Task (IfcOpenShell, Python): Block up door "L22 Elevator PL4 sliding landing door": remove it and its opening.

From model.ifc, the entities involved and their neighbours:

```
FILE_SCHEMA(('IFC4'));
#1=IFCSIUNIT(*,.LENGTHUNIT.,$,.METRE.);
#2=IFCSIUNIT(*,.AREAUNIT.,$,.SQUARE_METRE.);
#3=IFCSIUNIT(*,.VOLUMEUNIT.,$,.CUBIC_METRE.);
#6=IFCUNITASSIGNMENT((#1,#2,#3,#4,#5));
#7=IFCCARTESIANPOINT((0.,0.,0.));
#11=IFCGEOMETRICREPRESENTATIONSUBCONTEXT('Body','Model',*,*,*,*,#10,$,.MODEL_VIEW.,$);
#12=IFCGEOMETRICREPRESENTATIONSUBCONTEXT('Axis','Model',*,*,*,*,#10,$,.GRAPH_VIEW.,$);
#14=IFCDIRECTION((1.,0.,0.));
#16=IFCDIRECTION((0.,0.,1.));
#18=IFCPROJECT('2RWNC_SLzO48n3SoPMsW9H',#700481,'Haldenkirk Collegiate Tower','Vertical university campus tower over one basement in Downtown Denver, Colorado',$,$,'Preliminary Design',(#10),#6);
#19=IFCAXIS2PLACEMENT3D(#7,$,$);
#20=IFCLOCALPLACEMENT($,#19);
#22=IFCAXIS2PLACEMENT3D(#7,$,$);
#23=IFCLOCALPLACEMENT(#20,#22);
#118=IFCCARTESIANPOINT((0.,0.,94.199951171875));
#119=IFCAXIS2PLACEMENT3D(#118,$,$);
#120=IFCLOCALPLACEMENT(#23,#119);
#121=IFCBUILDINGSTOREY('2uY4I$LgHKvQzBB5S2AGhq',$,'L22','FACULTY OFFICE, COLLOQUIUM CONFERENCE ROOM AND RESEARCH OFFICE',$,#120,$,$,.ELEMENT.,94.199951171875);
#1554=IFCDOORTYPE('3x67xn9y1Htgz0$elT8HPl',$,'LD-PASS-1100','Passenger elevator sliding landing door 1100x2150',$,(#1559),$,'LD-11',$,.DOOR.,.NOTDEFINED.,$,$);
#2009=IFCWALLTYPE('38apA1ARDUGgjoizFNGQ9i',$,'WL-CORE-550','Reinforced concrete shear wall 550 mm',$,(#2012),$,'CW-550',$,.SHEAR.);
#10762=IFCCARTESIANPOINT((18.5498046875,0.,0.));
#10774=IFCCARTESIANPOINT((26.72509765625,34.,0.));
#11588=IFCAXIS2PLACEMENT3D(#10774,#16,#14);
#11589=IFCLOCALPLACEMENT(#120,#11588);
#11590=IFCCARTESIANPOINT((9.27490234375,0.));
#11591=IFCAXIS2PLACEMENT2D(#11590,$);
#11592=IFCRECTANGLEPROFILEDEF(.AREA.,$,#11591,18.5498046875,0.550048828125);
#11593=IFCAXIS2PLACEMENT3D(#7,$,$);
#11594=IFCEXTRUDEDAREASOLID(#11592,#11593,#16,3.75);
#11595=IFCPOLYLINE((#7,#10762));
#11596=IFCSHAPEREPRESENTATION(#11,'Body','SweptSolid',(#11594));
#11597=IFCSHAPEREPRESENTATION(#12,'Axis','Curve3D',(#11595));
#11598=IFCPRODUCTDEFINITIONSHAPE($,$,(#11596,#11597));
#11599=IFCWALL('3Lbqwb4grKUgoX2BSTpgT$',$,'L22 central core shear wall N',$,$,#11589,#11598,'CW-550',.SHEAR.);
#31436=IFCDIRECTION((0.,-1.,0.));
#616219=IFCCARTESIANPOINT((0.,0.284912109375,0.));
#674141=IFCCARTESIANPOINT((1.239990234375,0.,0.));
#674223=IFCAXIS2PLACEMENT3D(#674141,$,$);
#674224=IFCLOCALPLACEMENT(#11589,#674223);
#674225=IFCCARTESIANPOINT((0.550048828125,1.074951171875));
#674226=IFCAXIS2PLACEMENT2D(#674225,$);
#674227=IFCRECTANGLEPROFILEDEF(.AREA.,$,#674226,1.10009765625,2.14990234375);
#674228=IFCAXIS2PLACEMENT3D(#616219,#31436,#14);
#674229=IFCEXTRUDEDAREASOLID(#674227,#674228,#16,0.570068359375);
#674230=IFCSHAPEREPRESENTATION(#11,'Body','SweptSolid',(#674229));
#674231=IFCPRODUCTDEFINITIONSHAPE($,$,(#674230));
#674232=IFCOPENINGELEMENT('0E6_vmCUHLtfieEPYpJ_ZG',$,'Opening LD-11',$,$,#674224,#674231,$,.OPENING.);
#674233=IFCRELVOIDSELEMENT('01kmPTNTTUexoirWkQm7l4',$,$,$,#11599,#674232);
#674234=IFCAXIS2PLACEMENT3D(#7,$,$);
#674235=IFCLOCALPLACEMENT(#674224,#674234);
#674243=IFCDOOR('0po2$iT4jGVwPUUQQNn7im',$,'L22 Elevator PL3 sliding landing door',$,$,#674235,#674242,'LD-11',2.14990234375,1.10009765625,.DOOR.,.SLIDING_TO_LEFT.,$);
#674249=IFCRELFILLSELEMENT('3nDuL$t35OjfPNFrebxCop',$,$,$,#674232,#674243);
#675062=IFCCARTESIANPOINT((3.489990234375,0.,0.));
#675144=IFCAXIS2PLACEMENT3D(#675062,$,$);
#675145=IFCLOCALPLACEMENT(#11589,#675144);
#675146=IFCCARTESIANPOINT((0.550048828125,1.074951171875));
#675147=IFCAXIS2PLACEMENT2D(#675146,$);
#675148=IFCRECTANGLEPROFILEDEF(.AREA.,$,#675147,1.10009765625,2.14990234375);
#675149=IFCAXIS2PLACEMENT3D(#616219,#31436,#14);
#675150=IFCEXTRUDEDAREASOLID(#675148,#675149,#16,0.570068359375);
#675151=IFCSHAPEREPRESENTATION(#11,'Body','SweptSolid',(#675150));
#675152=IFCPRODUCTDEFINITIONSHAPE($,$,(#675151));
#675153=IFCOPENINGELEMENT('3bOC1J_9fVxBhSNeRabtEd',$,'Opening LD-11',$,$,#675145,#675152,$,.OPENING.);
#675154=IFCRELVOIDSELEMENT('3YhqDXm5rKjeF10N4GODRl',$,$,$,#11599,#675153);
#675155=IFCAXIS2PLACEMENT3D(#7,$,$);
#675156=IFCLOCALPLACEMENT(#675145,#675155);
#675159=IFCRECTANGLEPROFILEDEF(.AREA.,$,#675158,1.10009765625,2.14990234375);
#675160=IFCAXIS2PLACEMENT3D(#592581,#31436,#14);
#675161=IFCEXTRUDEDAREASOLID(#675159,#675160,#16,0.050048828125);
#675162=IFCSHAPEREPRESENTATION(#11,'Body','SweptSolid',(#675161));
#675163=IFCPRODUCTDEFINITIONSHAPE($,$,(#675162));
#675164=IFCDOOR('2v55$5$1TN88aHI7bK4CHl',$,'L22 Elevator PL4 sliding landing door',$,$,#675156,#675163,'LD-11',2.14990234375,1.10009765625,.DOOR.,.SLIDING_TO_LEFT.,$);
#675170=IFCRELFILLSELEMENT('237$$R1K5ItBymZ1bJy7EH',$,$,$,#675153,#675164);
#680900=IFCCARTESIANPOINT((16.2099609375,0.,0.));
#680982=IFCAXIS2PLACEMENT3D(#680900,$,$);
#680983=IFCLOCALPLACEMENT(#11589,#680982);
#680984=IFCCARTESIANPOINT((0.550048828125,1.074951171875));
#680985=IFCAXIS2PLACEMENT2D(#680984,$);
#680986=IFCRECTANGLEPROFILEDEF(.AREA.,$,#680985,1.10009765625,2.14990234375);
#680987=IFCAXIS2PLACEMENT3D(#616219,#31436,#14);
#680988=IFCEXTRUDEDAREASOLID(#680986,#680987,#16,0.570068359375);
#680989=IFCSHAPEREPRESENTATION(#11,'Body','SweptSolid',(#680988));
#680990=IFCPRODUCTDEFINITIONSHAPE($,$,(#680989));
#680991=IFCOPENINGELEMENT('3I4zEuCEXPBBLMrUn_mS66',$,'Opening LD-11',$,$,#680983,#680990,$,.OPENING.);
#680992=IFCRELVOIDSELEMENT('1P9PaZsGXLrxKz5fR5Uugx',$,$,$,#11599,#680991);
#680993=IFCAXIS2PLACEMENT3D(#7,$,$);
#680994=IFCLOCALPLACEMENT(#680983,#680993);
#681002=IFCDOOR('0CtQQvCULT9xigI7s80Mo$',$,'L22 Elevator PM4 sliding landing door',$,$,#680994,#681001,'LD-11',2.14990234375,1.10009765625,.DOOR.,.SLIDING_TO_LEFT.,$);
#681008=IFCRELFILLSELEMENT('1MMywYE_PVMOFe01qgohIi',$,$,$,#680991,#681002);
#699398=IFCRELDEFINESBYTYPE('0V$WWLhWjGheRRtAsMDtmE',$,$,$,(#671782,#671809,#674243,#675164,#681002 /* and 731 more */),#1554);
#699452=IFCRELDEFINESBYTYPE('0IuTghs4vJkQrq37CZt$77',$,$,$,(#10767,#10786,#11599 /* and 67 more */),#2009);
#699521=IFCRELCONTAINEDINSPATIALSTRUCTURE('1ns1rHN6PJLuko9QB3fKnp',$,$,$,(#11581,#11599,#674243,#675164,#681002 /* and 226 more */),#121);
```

```python
import ifcopenshell
import ifcopenshell.api.feature
import ifcopenshell.api.root
import ifcopenshell.geom
import ifcopenshell.util.shape

model = ifcopenshell.open("model.ifc")
settings = ifcopenshell.geom.settings()


def volume(element):
    """Net volume in cubic metres, openings subtracted."""
    shape = ifcopenshell.geom.create_shape(settings, element)
    return ifcopenshell.util.shape.get_volume(shape.geometry)


door = model.by_guid("2v55$5$1TN88aHI7bK4CHl")
opening = door.FillsVoids[0].RelatingOpeningElement
wall = opening.VoidsElements[0].RelatingBuildingElement
before = volume(wall)

ifcopenshell.api.root.remove_product(model, product=door)
ifcopenshell.api.feature.remove_feature(model, feature=opening)

after = volume(wall)

print(f"wall volume {before:.3f} -> {after:.3f} m3")

model.write("model_rev.ifc")
```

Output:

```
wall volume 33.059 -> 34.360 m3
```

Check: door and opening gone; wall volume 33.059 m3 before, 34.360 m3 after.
